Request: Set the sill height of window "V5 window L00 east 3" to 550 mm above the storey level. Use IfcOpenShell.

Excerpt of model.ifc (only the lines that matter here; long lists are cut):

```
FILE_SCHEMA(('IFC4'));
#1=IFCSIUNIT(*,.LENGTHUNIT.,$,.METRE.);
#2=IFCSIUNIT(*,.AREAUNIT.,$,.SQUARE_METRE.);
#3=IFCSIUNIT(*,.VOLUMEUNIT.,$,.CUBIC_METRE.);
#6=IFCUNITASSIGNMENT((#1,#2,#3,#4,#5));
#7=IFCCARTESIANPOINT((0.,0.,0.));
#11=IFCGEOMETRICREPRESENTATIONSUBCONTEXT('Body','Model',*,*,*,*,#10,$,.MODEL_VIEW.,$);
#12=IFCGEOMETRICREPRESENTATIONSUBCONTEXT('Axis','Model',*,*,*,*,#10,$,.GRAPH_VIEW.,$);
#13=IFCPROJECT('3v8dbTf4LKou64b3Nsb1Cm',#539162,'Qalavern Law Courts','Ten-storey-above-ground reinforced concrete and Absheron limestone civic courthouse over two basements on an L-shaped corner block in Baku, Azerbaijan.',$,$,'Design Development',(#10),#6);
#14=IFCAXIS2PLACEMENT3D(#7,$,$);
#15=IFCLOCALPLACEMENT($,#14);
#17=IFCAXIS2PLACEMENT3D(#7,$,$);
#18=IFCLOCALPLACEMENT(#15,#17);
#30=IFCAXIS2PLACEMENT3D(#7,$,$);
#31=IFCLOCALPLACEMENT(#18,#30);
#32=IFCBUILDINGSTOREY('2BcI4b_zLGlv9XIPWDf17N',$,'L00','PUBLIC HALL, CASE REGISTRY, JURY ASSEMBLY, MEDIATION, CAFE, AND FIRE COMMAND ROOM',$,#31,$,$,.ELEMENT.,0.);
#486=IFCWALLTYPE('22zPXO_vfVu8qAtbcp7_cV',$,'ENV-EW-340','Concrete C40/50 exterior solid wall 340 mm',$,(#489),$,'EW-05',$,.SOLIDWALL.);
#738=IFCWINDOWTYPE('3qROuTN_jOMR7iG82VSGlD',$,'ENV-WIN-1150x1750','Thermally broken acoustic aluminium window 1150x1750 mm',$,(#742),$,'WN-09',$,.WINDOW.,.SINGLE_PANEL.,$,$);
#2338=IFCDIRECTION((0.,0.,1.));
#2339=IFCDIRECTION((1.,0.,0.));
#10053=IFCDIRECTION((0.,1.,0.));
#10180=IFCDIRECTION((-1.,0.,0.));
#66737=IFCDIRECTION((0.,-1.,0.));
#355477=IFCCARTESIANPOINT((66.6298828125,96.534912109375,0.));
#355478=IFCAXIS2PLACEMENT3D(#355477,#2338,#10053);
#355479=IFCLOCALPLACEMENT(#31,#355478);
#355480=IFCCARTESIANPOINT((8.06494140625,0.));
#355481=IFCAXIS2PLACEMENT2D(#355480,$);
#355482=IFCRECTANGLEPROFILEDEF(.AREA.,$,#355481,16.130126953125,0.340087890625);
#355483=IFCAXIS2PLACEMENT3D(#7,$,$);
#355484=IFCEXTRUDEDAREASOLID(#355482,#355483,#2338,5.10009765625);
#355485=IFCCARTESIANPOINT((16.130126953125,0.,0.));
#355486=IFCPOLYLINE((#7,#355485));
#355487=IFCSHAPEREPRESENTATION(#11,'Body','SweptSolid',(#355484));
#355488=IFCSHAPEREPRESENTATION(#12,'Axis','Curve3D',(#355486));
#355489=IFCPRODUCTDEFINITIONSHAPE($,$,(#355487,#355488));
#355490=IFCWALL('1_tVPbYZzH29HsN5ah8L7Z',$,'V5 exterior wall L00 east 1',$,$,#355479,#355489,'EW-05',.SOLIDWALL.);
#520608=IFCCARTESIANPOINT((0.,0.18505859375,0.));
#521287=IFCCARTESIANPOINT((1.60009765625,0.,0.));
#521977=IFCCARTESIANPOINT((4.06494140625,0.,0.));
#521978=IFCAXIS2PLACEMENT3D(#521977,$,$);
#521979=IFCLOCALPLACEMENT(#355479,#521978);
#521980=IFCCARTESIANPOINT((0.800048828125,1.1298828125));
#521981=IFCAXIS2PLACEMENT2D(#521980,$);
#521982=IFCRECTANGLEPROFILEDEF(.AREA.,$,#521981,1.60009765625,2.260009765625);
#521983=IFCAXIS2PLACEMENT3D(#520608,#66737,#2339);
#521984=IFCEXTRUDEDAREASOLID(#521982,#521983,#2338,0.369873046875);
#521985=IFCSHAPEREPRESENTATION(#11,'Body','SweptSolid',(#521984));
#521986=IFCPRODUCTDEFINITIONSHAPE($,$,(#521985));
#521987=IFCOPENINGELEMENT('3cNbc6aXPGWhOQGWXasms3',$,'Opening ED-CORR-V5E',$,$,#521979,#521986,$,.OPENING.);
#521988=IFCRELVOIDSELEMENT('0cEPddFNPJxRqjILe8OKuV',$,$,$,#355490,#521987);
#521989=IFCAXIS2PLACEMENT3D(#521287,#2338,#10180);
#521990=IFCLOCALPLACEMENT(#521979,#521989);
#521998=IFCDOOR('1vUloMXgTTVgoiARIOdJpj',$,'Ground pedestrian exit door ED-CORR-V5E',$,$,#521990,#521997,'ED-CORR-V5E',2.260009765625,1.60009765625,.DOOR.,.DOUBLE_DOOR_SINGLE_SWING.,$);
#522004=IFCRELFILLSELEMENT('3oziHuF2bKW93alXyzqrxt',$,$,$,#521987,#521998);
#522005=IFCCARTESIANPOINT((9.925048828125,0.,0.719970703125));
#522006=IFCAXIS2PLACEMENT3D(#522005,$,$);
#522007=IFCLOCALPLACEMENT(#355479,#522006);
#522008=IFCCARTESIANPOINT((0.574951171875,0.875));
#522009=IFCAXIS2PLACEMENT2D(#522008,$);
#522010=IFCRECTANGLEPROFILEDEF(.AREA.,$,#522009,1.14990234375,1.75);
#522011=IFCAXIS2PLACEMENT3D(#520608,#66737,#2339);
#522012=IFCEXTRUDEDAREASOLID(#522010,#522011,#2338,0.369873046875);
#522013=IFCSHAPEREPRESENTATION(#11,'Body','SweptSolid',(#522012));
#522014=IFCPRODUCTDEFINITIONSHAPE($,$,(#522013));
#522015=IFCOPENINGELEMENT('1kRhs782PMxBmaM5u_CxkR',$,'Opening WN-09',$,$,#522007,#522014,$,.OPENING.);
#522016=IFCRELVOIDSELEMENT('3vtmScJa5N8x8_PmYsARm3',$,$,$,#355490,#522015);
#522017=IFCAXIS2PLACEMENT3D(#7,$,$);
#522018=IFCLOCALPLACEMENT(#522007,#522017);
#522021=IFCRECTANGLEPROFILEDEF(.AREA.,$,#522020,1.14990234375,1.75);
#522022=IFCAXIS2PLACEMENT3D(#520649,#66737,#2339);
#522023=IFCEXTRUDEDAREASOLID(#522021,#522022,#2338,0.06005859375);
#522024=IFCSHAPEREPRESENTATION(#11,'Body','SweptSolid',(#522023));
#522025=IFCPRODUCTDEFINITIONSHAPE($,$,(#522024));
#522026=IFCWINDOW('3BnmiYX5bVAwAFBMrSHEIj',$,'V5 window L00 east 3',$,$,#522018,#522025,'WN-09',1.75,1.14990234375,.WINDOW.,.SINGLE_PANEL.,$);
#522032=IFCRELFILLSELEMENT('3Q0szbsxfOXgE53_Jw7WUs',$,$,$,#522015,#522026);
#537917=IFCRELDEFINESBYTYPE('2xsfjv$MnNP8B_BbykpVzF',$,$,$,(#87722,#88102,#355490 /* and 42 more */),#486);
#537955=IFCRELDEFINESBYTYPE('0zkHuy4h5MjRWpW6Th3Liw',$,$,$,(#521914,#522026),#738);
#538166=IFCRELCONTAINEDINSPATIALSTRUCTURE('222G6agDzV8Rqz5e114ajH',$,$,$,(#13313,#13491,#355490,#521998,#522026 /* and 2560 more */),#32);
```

```python
import numpy as np
import ifcopenshell
import ifcopenshell.api.geometry
import ifcopenshell.geom
import ifcopenshell.util.element
import ifcopenshell.util.placement
import ifcopenshell.util.shape
import ifcopenshell.util.unit

model = ifcopenshell.open("model.ifc")
unit_scale = ifcopenshell.util.unit.calculate_unit_scale(model)

window = model.by_guid("3BnmiYX5bVAwAFBMrSHEIj")
opening = window.FillsVoids[0].RelatingOpeningElement
storey = ifcopenshell.util.element.get_container(window, ifc_class="IfcBuildingStorey")
level = ifcopenshell.util.placement.get_local_placement(storey.ObjectPlacement)[2, 3]

# The opening's origin need not be at the sill, so measure its lowest point.
shape = ifcopenshell.geom.create_shape(ifcopenshell.geom.settings(), opening)
bottom = ifcopenshell.util.shape.get_shape_bottom_elevation(shape, shape.geometry) / unit_scale
dz = level + 0.55 / unit_scale - bottom

shift = np.array([0.0, 0.0, dz])
# The window is placed relative to its opening, so it follows when the opening moves.
matrix = ifcopenshell.util.placement.get_local_placement(opening.ObjectPlacement)
matrix[:3, 3] += shift
ifcopenshell.api.geometry.edit_object_placement(
    model, product=opening, matrix=matrix, is_si=False, should_transform_children=True
)

print(f"moved by {dz * unit_scale:+.3f} m")

model.write("model-out.ifc")
```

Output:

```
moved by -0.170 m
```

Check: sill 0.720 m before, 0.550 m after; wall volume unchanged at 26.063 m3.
